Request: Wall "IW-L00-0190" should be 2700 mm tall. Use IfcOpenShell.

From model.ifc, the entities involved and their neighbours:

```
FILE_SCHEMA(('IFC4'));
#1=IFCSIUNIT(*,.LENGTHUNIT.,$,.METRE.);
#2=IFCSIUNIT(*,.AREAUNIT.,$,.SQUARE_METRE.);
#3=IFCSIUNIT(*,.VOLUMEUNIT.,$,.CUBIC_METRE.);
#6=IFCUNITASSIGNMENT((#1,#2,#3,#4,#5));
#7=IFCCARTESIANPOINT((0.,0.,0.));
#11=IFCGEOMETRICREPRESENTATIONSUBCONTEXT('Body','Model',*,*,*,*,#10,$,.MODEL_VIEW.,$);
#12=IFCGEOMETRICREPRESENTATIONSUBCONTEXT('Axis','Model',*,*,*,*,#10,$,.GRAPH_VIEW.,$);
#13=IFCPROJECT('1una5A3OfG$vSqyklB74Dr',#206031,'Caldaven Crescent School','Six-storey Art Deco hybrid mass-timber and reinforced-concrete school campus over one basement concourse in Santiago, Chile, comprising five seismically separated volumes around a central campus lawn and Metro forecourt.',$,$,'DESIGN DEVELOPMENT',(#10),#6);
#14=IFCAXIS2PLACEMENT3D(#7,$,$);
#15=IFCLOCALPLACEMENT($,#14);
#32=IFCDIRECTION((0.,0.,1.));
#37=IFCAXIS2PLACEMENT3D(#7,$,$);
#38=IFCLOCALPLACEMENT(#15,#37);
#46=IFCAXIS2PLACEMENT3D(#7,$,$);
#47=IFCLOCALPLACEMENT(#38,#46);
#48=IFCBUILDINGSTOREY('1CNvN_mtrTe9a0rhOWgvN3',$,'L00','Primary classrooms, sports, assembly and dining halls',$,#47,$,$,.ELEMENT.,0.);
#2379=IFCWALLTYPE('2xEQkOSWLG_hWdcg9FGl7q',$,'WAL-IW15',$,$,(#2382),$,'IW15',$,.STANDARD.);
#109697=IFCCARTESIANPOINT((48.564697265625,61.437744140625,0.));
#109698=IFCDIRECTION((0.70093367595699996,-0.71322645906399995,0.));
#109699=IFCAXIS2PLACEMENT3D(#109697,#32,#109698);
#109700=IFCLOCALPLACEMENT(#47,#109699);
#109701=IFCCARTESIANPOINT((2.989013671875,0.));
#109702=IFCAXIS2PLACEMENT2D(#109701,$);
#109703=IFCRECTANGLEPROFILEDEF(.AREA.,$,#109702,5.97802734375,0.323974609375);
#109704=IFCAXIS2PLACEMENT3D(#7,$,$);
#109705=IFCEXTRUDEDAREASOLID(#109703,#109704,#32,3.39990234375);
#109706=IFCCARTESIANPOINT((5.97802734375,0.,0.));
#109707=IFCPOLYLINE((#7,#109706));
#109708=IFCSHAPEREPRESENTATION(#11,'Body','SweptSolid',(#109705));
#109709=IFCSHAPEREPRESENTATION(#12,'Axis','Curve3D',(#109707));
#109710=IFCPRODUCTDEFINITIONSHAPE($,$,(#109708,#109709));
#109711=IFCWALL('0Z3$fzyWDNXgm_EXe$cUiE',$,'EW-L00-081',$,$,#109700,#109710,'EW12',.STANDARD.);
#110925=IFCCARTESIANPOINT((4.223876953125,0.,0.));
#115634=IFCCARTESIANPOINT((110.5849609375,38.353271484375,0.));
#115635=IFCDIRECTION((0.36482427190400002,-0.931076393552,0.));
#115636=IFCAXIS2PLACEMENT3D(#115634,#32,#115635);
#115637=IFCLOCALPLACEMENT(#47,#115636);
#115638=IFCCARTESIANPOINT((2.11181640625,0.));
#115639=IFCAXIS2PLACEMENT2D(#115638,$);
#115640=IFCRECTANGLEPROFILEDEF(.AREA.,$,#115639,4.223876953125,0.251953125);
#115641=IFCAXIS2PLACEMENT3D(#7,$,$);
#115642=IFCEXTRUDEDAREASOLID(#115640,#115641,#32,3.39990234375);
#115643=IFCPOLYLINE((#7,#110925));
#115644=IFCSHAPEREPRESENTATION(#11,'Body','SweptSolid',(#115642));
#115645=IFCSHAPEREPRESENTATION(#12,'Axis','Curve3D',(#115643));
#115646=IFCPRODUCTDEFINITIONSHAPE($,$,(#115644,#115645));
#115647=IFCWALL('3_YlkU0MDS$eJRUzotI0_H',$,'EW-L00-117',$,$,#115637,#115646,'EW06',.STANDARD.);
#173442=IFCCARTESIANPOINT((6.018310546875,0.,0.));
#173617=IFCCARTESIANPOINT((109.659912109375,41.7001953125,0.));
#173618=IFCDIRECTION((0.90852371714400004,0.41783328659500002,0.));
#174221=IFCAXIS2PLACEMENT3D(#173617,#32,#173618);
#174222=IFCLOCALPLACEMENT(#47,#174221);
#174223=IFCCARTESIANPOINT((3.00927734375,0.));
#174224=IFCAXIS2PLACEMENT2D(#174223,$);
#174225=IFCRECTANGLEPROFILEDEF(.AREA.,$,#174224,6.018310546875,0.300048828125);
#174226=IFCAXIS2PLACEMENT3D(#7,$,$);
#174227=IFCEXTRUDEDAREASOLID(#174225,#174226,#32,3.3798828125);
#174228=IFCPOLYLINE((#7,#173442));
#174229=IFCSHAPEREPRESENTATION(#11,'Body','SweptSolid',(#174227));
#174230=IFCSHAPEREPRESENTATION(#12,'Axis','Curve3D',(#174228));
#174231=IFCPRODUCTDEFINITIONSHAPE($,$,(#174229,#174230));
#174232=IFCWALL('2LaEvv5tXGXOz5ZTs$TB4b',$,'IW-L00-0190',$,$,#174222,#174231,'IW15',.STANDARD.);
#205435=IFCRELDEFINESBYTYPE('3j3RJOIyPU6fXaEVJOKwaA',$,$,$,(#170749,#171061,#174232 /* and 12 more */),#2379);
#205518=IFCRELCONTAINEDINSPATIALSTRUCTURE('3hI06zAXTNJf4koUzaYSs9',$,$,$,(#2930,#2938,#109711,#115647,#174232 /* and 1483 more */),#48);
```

```python
import ifcopenshell
import ifcopenshell.geom
import ifcopenshell.util.representation
import ifcopenshell.util.shape
import ifcopenshell.util.unit

model = ifcopenshell.open("model.ifc")
unit_scale = ifcopenshell.util.unit.calculate_unit_scale(model)
settings = ifcopenshell.geom.settings()


def volume(element):
    """Net volume in cubic metres, openings subtracted."""
    shape = ifcopenshell.geom.create_shape(settings, element)
    return ifcopenshell.util.shape.get_volume(shape.geometry)


wall = model.by_id(174232)
before = volume(wall)

body = ifcopenshell.util.representation.get_representation(wall, "Model", "Body")
solid = body.Items[0]
old_height = solid.Depth
solid.Depth = 2.7 / unit_scale
after = volume(wall)

print(f"height {old_height:g} -> {solid.Depth:g}, volume {before:.3f} -> {after:.3f} m3")

model.write("model-out.ifc")
```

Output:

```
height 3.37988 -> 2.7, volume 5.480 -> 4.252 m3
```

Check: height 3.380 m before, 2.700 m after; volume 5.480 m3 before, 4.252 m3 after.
